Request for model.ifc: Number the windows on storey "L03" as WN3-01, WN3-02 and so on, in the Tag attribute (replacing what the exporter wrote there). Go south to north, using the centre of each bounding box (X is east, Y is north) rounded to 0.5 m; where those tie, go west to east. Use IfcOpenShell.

First a look at what the model holds.

```python
import ifcopenshell
import ifcopenshell.util.element
import ifcopenshell.util.placement

model = ifcopenshell.open("model.ifc")
print(model.schema)
storey = next(s for s in model.by_type("IfcBuildingStorey") if s.Name == "L03")
windows = [e for e in ifcopenshell.util.element.get_decomposition(storey) if e.is_a("IfcWindow")]
for e in sorted(windows, key=lambda e: e.id()):
    origin = ifcopenshell.util.placement.get_local_placement(e.ObjectPlacement)[:3, 3]
    print(e.id(), e.Tag, e.Name, origin.round(2) + 0.0, sep=" | ")
```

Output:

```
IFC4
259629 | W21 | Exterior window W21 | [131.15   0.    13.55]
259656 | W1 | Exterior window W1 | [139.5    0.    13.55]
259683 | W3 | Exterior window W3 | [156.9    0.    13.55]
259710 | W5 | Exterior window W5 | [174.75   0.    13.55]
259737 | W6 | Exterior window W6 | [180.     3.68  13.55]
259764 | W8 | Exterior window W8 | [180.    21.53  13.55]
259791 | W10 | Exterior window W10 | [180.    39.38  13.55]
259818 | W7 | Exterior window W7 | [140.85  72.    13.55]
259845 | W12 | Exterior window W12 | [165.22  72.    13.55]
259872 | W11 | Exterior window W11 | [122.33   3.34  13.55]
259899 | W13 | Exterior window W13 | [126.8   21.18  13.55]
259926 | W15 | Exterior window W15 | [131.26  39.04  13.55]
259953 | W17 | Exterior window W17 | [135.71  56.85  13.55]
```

```python
import ifcopenshell
import ifcopenshell.geom
import ifcopenshell.util.element
import ifcopenshell.util.shape

model = ifcopenshell.open("model.ifc")
settings = ifcopenshell.geom.settings()
settings.set("use-world-coords", True)


def centre(element):
    shape = ifcopenshell.geom.create_shape(settings, element)
    return ifcopenshell.util.shape.get_bbox_centroid(shape.geometry)


storey = next(s for s in model.by_type("IfcBuildingStorey") if s.Name == "L03")
windows = [e for e in ifcopenshell.util.element.get_decomposition(storey) if e.is_a("IfcWindow")]

# Insertion points can sit at a corner or the storey origin, so sort by the geometry (in metres).
centres = {e: centre(e) for e in windows}
windows.sort(key=lambda e: (round(centres[e][1] / 0.5), centres[e][0]))

for i, e in enumerate(windows, start=1):
    number = f"WN3-{i:02d}"
    e.Tag = number
    print(e.id(), number)

model.write("model_edited.ifc")
```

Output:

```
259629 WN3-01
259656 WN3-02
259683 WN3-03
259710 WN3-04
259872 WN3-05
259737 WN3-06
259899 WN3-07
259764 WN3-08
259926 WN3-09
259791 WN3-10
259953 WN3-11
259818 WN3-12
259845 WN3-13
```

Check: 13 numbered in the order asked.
